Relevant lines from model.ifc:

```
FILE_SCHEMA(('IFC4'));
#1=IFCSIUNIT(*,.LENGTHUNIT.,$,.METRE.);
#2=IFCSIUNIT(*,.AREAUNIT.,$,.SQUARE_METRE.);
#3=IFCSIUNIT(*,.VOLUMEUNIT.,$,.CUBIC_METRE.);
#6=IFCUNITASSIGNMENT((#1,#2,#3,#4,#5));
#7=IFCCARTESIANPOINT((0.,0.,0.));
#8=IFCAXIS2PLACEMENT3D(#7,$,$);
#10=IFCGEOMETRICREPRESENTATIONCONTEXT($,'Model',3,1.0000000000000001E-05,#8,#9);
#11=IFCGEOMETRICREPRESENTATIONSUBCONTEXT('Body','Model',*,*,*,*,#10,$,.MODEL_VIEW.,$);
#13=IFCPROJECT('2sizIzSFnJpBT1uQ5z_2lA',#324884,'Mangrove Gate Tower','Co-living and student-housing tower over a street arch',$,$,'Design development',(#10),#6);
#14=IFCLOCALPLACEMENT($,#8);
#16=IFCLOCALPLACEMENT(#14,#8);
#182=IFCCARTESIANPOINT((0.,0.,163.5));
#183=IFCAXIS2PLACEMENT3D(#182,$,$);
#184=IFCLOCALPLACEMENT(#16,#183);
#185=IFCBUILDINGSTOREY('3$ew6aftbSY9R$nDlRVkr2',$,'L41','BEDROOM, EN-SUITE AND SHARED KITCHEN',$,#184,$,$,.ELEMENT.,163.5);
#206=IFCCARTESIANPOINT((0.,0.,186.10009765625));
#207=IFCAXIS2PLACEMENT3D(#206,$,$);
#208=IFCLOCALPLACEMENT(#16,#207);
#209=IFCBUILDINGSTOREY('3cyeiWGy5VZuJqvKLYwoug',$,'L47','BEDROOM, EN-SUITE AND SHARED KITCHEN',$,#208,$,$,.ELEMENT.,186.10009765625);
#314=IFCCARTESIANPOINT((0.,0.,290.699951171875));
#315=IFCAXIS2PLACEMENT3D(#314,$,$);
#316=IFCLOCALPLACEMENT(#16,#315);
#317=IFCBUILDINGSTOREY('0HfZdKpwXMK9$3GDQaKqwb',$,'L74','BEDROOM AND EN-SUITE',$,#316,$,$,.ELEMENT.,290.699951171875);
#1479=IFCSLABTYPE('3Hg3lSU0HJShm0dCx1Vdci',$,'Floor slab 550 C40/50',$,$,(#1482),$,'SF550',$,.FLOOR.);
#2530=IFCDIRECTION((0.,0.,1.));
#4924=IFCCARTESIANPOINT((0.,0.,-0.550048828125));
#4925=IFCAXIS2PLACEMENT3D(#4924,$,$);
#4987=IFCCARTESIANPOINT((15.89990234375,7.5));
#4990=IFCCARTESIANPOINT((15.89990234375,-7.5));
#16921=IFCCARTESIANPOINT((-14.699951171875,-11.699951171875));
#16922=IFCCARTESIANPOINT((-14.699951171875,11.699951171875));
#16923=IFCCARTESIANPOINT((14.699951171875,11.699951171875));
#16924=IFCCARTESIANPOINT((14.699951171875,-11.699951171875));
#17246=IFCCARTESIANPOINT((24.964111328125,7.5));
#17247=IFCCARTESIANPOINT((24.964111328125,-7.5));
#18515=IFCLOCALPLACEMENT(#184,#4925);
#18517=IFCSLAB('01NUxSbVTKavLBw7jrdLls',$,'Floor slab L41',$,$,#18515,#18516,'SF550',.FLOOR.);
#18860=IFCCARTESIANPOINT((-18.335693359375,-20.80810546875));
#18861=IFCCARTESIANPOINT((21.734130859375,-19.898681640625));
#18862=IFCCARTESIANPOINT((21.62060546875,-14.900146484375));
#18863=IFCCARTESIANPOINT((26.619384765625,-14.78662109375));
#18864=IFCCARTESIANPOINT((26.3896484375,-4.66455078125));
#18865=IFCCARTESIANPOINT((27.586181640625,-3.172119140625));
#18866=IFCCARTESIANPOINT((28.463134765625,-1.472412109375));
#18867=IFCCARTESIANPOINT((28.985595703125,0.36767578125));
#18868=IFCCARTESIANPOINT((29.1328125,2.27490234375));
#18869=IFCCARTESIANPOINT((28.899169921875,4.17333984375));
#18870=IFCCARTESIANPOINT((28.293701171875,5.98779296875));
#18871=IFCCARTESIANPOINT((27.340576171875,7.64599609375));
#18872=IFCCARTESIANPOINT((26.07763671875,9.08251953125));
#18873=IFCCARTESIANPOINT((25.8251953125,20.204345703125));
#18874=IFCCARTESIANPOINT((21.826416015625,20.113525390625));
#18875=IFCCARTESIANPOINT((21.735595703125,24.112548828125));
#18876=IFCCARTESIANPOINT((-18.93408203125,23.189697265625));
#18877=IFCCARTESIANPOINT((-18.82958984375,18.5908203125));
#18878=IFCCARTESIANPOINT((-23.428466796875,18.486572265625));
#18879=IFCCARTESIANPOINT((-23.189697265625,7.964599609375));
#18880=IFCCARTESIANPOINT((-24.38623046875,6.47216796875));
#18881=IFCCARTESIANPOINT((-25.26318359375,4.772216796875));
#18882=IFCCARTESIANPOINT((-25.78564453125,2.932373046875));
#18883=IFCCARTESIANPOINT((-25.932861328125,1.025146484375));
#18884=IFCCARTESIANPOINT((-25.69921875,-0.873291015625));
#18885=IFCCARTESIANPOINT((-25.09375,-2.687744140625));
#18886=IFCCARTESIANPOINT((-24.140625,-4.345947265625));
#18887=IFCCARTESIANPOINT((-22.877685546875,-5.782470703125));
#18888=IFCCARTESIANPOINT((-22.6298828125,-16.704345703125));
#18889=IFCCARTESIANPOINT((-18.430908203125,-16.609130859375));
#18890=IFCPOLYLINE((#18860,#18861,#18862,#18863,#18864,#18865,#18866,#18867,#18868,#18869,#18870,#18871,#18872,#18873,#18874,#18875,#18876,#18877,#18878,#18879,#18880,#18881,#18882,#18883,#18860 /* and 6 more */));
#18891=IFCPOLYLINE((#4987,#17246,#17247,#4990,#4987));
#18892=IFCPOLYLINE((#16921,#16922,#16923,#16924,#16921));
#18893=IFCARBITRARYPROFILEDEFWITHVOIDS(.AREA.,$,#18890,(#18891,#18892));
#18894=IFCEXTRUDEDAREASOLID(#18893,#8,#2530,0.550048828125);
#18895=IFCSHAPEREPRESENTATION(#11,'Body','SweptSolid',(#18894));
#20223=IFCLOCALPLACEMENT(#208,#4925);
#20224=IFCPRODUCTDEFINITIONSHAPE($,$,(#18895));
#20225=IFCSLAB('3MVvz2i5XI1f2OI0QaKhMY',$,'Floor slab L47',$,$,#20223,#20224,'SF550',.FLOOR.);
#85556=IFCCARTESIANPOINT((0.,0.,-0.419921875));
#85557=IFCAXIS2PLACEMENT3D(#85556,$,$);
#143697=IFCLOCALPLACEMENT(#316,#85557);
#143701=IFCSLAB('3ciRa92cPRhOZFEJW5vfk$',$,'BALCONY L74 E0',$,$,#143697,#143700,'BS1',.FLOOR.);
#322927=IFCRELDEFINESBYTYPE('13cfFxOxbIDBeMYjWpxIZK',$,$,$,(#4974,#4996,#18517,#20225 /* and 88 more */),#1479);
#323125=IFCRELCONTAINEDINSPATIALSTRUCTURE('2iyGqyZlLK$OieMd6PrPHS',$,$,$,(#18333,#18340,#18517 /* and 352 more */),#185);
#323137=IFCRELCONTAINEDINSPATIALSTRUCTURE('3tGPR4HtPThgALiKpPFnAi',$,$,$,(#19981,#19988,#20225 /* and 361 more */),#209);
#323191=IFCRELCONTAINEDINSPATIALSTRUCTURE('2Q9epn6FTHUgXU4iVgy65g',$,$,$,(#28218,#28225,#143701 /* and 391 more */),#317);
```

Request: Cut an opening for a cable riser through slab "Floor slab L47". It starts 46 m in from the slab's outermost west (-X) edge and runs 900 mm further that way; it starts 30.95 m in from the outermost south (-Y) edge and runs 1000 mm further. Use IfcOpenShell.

```python
import numpy as np
import ifcopenshell
import ifcopenshell.api.feature
import ifcopenshell.api.geometry
import ifcopenshell.api.root
import ifcopenshell.geom
import ifcopenshell.util.placement
import ifcopenshell.util.representation
import ifcopenshell.util.shape
import ifcopenshell.util.unit

model = ifcopenshell.open("model.ifc")
unit_scale = ifcopenshell.util.unit.calculate_unit_scale(model)
settings = ifcopenshell.geom.settings()


def volume(element):
    """Net volume in cubic metres, openings subtracted."""
    shape = ifcopenshell.geom.create_shape(settings, element)
    return ifcopenshell.util.shape.get_volume(shape.geometry)


slab = model.by_guid("3MVvz2i5XI1f2OI0QaKhMY")
before = volume(slab)

# Extent in the slab's own axes, in metres. The edges named are its -X and -Y sides.
slab_shape = ifcopenshell.geom.create_shape(settings, slab)
vertices = ifcopenshell.util.shape.get_vertices(slab_shape.geometry)
x_min, y_min, bottom = vertices.min(axis=0)
top = vertices[:, 2].max()

opening = ifcopenshell.api.root.create_entity(model, ifc_class="IfcOpeningElement", name="Cable riser opening", predefined_type="OPENING")
context = ifcopenshell.util.representation.get_context(model, "Model", "Body", "MODEL_VIEW")
width, depth = 0.9, 1
outline = [(0.0, 0.0), (width, 0.0), (width, depth), (0.0, depth), (0.0, 0.0)]
# Overshoot both faces by 50 mm so the cut is clean.
shape = ifcopenshell.api.geometry.add_slab_representation(
    model, context=context, depth=top - bottom + 0.1, polyline=outline
)
ifcopenshell.api.geometry.assign_representation(model, product=opening, representation=shape)

matrix = ifcopenshell.util.placement.get_local_placement(slab.ObjectPlacement)
matrix[:, 3] = matrix @ np.append(np.array([x_min + 46, y_min + 30.95, bottom - 0.05]) / unit_scale, 1.0)
ifcopenshell.api.geometry.edit_object_placement(model, product=opening, matrix=matrix, is_si=False)
ifcopenshell.api.feature.add_feature(model, feature=opening, element=slab)

after = volume(slab)

print(f"slab volume {before:.3f} -> {after:.3f} m3")

model.write("model_v2.ifc")
```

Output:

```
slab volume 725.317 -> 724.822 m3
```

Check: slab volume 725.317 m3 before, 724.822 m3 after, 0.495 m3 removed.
